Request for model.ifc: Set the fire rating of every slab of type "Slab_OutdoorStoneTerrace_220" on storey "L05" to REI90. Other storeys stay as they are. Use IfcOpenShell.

First a look at what the model holds.

```python
import ifcopenshell
import ifcopenshell.util.element

model = ifcopenshell.open("model.ifc")
print(model.schema)
storey = next(s for s in model.by_type("IfcBuildingStorey") if s.Name == "L05")
slabs = [e for e in ifcopenshell.util.element.get_decomposition(storey) if e.is_a("IfcSlab")]
seen = {}
for e in slabs:
    element_type = ifcopenshell.util.element.get_type(e)
    key = (element_type.Name if element_type != e and element_type else None, ifcopenshell.util.element.get_pset(e, "Pset_SlabCommon", "FireRating"))
    seen[key] = seen.get(key, 0) + 1
for (name, value), count in sorted(seen.items(), key=str):
    print(count, "x", name, "|", value)
```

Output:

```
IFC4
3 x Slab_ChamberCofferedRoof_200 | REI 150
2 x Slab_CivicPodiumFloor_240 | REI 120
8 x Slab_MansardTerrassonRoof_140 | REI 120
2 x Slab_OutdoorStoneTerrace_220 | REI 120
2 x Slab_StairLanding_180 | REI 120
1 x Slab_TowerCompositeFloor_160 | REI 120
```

```python
import ifcopenshell
import ifcopenshell.api.pset
import ifcopenshell.util.element

model = ifcopenshell.open("model.ifc")

storey = next(s for s in model.by_type("IfcBuildingStorey") if s.Name == "L05")
slabs = [e for e in ifcopenshell.util.element.get_decomposition(storey) if e.is_a("IfcSlab")]

count = 0
for e in slabs:
    element_type = ifcopenshell.util.element.get_type(e)
    if element_type in (None, e) or element_type.Name != "Slab_OutdoorStoneTerrace_220":
        continue
    # add_pset returns the element's existing set when there is one.
    pset = ifcopenshell.api.pset.add_pset(model, product=e, name="Pset_SlabCommon")
    ifcopenshell.api.pset.edit_pset(model, pset=pset, properties={"FireRating": "REI90"})
    count += 1

print(count, "slabs updated")

model.write("model-out.ifc")
```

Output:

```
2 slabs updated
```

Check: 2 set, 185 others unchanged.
